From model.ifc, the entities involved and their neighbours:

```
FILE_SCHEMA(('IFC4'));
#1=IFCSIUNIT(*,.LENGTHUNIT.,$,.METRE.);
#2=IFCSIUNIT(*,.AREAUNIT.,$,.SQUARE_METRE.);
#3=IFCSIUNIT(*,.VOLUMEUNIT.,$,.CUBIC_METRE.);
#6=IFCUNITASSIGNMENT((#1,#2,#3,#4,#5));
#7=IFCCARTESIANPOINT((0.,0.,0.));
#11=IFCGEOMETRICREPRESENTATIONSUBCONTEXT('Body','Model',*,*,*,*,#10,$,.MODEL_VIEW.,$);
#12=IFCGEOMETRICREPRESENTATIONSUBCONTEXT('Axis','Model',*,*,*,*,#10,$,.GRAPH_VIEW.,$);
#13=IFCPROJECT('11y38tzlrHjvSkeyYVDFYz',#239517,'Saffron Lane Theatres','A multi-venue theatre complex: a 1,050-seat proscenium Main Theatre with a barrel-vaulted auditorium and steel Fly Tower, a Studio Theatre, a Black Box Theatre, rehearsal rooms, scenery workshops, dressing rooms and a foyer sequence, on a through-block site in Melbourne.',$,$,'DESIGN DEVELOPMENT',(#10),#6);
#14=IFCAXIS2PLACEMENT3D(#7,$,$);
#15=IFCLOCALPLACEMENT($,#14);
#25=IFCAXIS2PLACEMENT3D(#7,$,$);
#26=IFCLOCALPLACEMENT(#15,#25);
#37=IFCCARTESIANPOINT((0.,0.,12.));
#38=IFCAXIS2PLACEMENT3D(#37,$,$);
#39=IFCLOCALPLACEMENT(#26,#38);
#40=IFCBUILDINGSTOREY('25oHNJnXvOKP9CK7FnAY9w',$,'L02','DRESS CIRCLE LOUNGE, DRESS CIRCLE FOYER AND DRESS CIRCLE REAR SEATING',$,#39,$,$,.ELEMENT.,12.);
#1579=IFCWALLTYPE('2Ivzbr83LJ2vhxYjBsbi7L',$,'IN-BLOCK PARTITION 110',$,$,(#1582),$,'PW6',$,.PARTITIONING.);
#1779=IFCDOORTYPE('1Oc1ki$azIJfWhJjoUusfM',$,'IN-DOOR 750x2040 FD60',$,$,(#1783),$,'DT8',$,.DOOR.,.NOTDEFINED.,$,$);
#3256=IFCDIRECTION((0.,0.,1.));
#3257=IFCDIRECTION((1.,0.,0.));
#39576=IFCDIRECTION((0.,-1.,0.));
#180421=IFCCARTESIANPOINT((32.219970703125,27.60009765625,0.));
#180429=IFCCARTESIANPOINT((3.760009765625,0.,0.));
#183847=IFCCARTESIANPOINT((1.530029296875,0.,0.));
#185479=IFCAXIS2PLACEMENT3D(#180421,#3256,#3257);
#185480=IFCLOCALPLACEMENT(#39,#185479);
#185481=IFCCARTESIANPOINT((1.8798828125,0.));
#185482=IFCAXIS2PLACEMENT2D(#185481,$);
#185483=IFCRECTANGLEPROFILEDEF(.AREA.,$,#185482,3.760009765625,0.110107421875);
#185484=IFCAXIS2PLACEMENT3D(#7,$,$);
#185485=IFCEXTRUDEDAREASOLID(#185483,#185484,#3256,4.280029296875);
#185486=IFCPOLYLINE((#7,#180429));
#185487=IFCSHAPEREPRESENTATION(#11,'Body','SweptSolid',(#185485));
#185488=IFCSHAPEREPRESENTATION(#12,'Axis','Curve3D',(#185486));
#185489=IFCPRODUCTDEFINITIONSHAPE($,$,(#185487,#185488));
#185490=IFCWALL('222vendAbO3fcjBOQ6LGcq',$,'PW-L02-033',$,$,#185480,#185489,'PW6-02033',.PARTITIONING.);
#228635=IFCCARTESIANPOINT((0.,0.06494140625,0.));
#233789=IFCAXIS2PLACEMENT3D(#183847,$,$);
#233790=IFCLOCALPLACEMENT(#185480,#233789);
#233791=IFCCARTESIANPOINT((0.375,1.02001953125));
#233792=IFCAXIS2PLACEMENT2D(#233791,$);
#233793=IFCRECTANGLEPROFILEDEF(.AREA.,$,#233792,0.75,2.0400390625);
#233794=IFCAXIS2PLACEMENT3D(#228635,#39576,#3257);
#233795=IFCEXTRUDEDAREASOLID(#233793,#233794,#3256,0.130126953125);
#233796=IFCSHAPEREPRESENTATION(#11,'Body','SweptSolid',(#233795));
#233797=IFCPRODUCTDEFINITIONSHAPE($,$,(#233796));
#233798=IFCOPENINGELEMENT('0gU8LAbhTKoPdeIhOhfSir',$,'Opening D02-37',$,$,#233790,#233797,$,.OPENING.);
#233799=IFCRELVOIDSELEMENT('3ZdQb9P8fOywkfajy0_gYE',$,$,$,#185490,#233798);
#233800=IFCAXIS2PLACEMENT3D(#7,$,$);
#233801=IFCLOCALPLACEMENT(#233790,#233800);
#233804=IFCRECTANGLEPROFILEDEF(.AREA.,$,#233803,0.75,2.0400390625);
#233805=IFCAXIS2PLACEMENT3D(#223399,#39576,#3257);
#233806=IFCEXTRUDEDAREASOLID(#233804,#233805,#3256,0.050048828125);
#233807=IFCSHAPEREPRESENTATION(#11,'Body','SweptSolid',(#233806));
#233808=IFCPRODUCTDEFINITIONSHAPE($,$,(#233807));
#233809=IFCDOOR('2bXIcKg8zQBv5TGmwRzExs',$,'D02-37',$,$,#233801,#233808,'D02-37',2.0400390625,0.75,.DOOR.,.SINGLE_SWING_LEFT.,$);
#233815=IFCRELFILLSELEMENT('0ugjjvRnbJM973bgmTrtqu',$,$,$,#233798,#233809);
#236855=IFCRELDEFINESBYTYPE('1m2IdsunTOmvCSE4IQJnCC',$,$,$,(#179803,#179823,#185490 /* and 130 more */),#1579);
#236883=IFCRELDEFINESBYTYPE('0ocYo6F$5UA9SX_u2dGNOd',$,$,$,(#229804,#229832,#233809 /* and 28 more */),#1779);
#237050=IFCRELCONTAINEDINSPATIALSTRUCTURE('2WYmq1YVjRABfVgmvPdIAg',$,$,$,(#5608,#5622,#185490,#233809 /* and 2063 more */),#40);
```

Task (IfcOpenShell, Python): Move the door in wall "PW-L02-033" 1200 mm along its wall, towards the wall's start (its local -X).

```python
import ifcopenshell
import ifcopenshell.api.geometry
import ifcopenshell.util.placement

model = ifcopenshell.open("model.ifc")

door = model.by_guid("2bXIcKg8zQBv5TGmwRzExs")
opening = door.FillsVoids[0].RelatingOpeningElement
wall = opening.VoidsElements[0].RelatingBuildingElement

wall_matrix = ifcopenshell.util.placement.get_local_placement(wall.ObjectPlacement)
shift = wall_matrix[:3, 0] * -1.2
before = ifcopenshell.util.placement.get_local_placement(door.ObjectPlacement)[:3, 3].copy()

# The door is placed relative to its opening, so it follows when the opening moves.
matrix = ifcopenshell.util.placement.get_local_placement(opening.ObjectPlacement)
matrix[:3, 3] += shift
ifcopenshell.api.geometry.edit_object_placement(
    model, product=opening, matrix=matrix, is_si=False, should_transform_children=True
)

after = ifcopenshell.util.placement.get_local_placement(door.ObjectPlacement)[:3, 3]
print("door moved by", (after - before).round(3) + 0.0)

model.write("model_v2.ifc")
```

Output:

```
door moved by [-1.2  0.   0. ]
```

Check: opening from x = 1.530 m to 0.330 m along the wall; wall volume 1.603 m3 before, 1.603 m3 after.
